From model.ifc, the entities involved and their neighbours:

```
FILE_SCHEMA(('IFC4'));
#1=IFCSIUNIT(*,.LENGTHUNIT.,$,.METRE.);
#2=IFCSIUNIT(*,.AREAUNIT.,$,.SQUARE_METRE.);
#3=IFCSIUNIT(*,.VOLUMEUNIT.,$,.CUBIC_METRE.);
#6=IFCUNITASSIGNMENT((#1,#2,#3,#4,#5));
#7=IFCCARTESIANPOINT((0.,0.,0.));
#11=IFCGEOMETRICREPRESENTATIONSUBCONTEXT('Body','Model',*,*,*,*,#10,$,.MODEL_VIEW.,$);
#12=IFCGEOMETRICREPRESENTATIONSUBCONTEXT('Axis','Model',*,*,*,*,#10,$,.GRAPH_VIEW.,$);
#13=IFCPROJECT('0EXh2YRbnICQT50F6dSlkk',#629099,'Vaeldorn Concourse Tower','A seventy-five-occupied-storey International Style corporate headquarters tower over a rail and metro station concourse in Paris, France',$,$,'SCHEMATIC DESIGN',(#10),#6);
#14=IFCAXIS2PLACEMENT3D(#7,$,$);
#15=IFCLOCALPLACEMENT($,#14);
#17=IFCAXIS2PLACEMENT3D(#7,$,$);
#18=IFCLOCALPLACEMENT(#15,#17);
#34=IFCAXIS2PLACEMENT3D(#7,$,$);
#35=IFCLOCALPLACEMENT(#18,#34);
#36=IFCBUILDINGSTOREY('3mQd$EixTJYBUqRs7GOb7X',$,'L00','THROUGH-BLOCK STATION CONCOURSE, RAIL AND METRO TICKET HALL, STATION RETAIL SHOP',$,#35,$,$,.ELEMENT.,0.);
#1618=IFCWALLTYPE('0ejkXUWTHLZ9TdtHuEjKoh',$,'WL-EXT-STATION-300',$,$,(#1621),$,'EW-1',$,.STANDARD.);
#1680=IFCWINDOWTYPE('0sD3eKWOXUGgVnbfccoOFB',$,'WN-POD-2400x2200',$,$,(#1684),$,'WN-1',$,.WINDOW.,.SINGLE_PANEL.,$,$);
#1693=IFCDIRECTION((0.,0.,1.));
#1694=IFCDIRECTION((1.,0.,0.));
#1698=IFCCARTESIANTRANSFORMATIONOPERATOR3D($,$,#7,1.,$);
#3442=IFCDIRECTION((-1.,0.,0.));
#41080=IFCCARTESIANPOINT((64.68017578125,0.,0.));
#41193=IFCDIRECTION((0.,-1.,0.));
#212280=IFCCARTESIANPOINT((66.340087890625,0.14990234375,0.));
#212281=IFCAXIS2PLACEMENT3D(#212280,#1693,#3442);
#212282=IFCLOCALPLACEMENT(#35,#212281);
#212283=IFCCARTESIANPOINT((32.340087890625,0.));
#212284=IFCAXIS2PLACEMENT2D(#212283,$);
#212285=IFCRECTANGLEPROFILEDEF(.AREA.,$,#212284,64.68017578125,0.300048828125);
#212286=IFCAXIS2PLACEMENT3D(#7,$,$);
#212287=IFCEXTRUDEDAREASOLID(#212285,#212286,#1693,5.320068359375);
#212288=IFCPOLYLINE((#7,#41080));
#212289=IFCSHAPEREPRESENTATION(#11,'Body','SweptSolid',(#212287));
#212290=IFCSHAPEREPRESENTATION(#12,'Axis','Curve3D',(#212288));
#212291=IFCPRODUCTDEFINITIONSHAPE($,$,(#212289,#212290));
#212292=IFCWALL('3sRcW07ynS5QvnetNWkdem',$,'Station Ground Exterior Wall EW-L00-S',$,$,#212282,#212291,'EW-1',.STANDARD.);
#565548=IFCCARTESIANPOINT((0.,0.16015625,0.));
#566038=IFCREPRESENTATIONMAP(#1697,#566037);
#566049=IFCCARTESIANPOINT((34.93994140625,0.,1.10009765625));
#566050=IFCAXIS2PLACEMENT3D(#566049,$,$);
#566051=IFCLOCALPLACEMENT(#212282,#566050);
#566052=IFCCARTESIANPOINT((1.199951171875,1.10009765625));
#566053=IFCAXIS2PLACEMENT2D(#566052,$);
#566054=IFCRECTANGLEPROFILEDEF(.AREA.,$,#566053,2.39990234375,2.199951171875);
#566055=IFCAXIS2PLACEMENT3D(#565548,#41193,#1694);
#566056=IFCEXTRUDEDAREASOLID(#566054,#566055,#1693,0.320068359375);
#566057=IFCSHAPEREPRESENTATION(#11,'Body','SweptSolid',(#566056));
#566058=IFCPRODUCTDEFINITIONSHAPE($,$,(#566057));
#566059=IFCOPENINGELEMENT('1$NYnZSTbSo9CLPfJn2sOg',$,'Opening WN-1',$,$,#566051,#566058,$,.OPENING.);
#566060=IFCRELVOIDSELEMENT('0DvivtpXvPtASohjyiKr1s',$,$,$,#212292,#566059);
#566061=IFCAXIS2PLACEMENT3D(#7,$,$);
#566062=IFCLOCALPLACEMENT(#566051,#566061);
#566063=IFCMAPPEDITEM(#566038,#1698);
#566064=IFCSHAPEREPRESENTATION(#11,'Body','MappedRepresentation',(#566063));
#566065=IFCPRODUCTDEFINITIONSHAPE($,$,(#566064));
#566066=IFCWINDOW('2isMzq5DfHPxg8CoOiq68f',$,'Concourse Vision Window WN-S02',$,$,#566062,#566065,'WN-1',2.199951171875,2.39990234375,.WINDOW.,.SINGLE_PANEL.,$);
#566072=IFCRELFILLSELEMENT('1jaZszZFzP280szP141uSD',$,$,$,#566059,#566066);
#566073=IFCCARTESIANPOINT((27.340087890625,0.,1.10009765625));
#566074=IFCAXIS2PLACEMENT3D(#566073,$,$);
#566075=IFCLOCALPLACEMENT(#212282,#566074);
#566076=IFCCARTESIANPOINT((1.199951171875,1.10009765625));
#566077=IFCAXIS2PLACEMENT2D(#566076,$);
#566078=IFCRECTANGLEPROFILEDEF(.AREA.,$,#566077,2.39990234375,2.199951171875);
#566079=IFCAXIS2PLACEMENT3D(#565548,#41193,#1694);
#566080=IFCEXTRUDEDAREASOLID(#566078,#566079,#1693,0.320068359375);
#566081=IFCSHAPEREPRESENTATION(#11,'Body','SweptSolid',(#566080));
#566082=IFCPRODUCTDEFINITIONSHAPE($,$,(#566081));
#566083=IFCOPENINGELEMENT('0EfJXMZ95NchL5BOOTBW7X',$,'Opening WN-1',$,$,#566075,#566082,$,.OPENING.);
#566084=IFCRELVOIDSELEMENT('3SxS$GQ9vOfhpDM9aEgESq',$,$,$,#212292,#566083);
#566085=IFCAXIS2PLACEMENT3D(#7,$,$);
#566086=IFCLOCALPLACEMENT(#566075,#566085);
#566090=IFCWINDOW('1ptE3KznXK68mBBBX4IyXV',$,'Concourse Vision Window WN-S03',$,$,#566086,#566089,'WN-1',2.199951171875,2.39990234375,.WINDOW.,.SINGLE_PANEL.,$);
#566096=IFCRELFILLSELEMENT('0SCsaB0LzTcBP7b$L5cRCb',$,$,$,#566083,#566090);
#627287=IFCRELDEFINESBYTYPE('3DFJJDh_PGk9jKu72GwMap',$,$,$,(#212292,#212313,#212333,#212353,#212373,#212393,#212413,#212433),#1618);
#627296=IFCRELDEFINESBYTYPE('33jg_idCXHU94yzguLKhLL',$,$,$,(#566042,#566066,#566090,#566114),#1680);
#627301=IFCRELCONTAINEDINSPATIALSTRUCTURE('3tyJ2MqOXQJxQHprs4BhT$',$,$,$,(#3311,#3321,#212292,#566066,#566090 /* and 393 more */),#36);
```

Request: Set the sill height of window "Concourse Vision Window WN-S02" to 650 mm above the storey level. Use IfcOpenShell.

```python
import numpy as np
import ifcopenshell
import ifcopenshell.api.geometry
import ifcopenshell.geom
import ifcopenshell.util.element
import ifcopenshell.util.placement
import ifcopenshell.util.shape
import ifcopenshell.util.unit

model = ifcopenshell.open("model.ifc")
unit_scale = ifcopenshell.util.unit.calculate_unit_scale(model)

window = model.by_guid("2isMzq5DfHPxg8CoOiq68f")
opening = window.FillsVoids[0].RelatingOpeningElement
storey = ifcopenshell.util.element.get_container(window, ifc_class="IfcBuildingStorey")
level = ifcopenshell.util.placement.get_local_placement(storey.ObjectPlacement)[2, 3]

# The opening's origin need not be at the sill, so measure its lowest point.
shape = ifcopenshell.geom.create_shape(ifcopenshell.geom.settings(), opening)
bottom = ifcopenshell.util.shape.get_shape_bottom_elevation(shape, shape.geometry) / unit_scale
dz = level + 0.65 / unit_scale - bottom

shift = np.array([0.0, 0.0, dz])
# The window is placed relative to its opening, so it follows when the opening moves.
matrix = ifcopenshell.util.placement.get_local_placement(opening.ObjectPlacement)
matrix[:3, 3] += shift
ifcopenshell.api.geometry.edit_object_placement(
    model, product=opening, matrix=matrix, is_si=False, should_transform_children=True
)

print(f"moved by {dz * unit_scale:+.3f} m")

model.write("model_edited.ifc")
```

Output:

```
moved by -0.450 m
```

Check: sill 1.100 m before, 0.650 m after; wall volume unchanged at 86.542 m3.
